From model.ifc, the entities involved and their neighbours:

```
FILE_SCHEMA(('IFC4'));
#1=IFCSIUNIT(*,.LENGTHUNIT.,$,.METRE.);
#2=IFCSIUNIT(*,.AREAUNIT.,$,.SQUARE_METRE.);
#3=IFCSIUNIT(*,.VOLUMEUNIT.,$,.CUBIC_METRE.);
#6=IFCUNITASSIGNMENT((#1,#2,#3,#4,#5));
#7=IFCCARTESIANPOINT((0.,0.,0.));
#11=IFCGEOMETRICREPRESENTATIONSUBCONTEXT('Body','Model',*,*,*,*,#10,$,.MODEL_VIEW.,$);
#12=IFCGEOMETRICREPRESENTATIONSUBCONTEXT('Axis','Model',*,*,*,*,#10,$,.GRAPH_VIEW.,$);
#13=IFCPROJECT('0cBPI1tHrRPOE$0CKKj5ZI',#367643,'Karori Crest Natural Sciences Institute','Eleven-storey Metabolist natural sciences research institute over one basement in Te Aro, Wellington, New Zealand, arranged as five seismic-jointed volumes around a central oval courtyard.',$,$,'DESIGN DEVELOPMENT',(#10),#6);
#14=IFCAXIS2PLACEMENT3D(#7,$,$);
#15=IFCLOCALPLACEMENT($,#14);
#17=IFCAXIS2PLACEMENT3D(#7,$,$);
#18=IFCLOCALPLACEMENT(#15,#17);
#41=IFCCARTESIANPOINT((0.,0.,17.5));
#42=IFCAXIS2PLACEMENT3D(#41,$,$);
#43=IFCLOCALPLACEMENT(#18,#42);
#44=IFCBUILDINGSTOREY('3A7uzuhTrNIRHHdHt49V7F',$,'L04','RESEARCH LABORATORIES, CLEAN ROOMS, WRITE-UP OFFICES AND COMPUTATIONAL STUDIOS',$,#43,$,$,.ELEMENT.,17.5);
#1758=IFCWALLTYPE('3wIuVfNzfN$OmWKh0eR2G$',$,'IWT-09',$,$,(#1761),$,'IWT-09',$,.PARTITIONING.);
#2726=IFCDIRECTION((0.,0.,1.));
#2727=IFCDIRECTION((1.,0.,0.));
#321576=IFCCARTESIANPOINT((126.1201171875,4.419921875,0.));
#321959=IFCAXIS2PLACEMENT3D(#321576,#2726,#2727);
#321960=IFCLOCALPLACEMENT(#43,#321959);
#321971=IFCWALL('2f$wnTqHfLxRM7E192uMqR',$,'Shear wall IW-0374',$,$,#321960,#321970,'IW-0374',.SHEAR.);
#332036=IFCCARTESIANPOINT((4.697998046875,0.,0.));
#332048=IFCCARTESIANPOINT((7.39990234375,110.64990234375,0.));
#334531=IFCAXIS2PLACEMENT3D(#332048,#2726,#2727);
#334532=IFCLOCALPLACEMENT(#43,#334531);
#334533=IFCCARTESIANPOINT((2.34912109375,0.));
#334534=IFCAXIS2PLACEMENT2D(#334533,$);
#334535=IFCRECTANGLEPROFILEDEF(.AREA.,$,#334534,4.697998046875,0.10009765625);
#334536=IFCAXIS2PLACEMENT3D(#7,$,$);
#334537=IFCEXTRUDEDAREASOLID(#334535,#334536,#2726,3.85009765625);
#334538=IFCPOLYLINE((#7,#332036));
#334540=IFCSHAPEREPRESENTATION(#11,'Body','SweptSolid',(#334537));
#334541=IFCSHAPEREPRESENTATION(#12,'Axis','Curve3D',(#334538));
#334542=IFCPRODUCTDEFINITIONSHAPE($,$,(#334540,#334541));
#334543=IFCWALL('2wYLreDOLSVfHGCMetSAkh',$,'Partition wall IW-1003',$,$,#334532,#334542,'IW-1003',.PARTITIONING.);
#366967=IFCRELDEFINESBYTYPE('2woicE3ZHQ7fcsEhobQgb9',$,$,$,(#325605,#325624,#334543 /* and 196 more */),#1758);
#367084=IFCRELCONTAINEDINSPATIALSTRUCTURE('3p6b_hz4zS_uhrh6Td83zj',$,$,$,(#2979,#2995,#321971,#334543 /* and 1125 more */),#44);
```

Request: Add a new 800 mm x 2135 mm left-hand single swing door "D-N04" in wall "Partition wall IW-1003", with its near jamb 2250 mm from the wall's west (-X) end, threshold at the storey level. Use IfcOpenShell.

```python
import numpy as np
import ifcopenshell
import ifcopenshell.api.feature
import ifcopenshell.api.geometry
import ifcopenshell.api.root
import ifcopenshell.api.spatial
import ifcopenshell.geom
import ifcopenshell.util.element
import ifcopenshell.util.placement
import ifcopenshell.util.representation
import ifcopenshell.util.shape
import ifcopenshell.util.unit

model = ifcopenshell.open("model.ifc")
unit_scale = ifcopenshell.util.unit.calculate_unit_scale(model)
settings = ifcopenshell.geom.settings()


def volume(element):
    """Net volume in cubic metres, openings subtracted."""
    shape = ifcopenshell.geom.create_shape(settings, element)
    return ifcopenshell.util.shape.get_volume(shape.geometry)


wall = model.by_guid("2wYLreDOLSVfHGCMetSAkh")
storey = ifcopenshell.util.element.get_container(wall, ifc_class="IfcBuildingStorey")
context = ifcopenshell.util.representation.get_context(model, "Model", "Body", "MODEL_VIEW")
before = volume(wall)

width, height, from_end, sill = 0.8, 2.135, 2.25, 0.0  # metres

# The wall runs along its own X axis, and the end named is its -X end.
wall_shape = ifcopenshell.geom.create_shape(settings, wall)
x, y, z = ifcopenshell.util.shape.get_vertices(wall_shape.geometry).T
start = x.min() + from_end
face, thickness = float(y.min()), float(y.max() - y.min())
wall_matrix = ifcopenshell.util.placement.get_local_placement(wall.ObjectPlacement)
level = ifcopenshell.util.placement.get_local_placement(storey.ObjectPlacement)[2, 3]


def in_wall(x, y):
    """Placement at x, y metres in the wall's axes, at sill height."""
    matrix = wall_matrix.copy()
    matrix[:, 3] = wall_matrix @ np.array([x / unit_scale, y / unit_scale, 0.0, 1.0])
    matrix[2, 3] = level + sill / unit_scale
    return matrix


# Opening: a box that overshoots both wall faces by 50 mm.
opening = ifcopenshell.api.root.create_entity(model, ifc_class="IfcOpeningElement", predefined_type="OPENING")
box = ifcopenshell.api.geometry.add_wall_representation(
    model, context=context, length=width, height=height, thickness=thickness + 0.1
)
ifcopenshell.api.geometry.assign_representation(model, product=opening, representation=box)
ifcopenshell.api.geometry.edit_object_placement(model, product=opening, matrix=in_wall(start, face - 0.05), is_si=False)
ifcopenshell.api.feature.add_feature(model, feature=opening, element=wall)

door = ifcopenshell.api.root.create_entity(model, ifc_class="IfcDoor", name="D-N04", predefined_type="DOOR")
door.OverallWidth, door.OverallHeight = width / unit_scale, height / unit_scale
door.OperationType = "SINGLE_SWING_LEFT"
body = ifcopenshell.api.geometry.add_door_representation(
    model,
    context=context,
    overall_width=door.OverallWidth,
    overall_height=door.OverallHeight,
    operation_type="SINGLE_SWING_LEFT",
    lining_properties={"LiningDepth": thickness / unit_scale, "ThresholdDepth": thickness / unit_scale},
)
ifcopenshell.api.geometry.assign_representation(model, product=door, representation=body)
ifcopenshell.api.spatial.assign_container(model, products=[door], relating_structure=storey)
ifcopenshell.api.feature.add_filling(model, opening=opening, element=door)

# The lining spans the wall, so the door starts at the wall face.
ifcopenshell.api.geometry.edit_object_placement(model, product=door, matrix=in_wall(start, face), is_si=False)

after = volume(wall)

print(f"wall volume {before:.3f} -> {after:.3f} m3")

model.write("model_updated.ifc")
```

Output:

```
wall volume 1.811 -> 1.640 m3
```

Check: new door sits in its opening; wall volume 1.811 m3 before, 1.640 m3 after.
